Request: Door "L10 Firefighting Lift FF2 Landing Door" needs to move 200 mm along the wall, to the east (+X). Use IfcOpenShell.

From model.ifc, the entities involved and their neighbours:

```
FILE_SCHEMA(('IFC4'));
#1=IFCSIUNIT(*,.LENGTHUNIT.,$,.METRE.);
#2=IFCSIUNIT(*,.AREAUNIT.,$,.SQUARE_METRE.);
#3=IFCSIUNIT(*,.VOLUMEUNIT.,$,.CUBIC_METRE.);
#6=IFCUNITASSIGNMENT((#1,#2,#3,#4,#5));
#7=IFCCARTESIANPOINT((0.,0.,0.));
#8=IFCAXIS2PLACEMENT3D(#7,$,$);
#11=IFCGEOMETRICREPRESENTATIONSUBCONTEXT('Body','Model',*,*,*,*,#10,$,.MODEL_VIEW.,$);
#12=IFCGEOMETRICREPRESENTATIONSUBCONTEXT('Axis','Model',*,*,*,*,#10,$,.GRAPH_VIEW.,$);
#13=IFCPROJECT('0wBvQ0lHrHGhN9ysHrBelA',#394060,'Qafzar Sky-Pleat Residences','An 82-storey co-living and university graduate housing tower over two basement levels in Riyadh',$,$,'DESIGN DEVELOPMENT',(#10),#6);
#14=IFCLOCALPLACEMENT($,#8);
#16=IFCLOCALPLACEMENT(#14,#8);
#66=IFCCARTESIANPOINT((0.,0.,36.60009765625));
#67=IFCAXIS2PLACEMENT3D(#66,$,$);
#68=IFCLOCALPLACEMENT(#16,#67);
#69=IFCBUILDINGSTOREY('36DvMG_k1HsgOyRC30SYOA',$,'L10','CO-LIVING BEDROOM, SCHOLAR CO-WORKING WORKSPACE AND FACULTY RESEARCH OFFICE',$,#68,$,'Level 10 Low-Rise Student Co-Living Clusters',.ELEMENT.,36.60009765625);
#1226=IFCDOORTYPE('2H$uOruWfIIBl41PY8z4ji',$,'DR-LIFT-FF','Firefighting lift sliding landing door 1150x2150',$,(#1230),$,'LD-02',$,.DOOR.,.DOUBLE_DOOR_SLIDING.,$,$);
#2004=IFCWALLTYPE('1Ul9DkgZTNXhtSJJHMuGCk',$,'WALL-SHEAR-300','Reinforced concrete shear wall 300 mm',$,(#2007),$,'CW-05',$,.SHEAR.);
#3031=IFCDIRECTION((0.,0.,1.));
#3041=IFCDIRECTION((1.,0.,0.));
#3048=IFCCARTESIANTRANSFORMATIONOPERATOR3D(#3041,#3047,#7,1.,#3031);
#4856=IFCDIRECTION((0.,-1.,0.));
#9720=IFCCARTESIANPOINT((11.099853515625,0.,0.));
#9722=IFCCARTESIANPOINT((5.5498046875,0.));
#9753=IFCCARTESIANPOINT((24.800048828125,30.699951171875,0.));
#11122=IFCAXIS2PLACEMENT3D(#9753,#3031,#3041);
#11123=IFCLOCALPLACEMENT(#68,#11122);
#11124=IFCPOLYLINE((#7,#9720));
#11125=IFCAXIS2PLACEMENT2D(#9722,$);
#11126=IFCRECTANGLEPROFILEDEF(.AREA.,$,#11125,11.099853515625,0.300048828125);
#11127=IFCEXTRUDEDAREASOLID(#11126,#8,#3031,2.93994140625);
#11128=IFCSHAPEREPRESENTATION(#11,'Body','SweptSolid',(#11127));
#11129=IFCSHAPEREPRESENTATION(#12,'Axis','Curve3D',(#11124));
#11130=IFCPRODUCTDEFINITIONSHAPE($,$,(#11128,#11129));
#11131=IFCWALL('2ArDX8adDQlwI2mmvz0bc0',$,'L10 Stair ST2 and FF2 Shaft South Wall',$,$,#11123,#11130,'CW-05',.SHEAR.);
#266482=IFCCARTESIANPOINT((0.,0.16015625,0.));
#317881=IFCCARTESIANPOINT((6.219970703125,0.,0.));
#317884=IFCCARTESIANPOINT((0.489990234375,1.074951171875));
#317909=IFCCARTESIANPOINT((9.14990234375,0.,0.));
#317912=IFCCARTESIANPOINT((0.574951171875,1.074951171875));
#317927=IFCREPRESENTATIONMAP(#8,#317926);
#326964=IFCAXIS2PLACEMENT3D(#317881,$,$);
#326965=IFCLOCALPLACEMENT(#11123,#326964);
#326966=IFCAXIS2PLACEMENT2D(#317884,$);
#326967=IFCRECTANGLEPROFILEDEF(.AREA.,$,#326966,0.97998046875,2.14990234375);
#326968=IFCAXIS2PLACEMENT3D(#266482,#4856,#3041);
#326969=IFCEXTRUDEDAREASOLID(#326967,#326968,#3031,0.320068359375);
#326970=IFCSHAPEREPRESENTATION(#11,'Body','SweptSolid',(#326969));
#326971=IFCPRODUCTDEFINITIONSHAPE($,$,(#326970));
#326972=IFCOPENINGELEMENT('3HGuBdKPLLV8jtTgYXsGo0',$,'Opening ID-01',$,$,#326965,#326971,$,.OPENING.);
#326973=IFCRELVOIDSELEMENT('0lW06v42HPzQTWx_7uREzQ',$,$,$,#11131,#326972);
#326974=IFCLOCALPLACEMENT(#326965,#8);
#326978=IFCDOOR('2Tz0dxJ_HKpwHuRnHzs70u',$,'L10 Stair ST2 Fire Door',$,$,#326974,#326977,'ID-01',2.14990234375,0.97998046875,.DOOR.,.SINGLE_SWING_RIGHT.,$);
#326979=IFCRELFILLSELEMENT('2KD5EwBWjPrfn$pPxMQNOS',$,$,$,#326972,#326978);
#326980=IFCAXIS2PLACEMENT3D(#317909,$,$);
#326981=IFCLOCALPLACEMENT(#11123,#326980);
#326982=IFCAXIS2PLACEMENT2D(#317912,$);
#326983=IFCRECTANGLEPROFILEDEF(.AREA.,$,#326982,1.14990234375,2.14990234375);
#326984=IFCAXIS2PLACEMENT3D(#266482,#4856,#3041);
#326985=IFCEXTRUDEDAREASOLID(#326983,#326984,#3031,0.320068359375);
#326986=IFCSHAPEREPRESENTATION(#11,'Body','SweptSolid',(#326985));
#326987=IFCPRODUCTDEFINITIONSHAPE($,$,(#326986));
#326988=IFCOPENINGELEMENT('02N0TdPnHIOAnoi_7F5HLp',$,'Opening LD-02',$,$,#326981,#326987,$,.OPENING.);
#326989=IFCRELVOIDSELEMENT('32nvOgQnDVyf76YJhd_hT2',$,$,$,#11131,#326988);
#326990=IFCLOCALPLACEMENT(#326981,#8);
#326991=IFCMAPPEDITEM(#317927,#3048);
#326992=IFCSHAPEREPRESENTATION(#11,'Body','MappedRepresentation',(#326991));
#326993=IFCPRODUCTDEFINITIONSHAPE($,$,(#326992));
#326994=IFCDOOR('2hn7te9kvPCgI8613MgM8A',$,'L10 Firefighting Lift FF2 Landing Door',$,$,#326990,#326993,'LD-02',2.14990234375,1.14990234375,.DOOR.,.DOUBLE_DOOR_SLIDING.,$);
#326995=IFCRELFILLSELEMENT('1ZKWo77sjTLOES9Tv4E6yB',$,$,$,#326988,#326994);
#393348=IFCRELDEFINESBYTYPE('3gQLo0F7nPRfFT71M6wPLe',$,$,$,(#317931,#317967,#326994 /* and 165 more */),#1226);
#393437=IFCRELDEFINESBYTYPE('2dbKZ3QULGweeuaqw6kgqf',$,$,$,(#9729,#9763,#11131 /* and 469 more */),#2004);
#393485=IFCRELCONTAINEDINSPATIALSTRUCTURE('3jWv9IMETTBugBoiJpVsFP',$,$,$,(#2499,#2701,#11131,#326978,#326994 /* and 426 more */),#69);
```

```python
import ifcopenshell
import ifcopenshell.api.geometry
import ifcopenshell.util.placement
import ifcopenshell.util.unit

model = ifcopenshell.open("model.ifc")
unit_scale = ifcopenshell.util.unit.calculate_unit_scale(model)

door = model.by_guid("2hn7te9kvPCgI8613MgM8A")
opening = door.FillsVoids[0].RelatingOpeningElement
wall = opening.VoidsElements[0].RelatingBuildingElement

wall_matrix = ifcopenshell.util.placement.get_local_placement(wall.ObjectPlacement)
shift = wall_matrix[:3, 0] * 0.2 / unit_scale
before = ifcopenshell.util.placement.get_local_placement(door.ObjectPlacement)[:3, 3].copy()

# The door is placed relative to its opening, so it follows when the opening moves.
matrix = ifcopenshell.util.placement.get_local_placement(opening.ObjectPlacement)
matrix[:3, 3] += shift
ifcopenshell.api.geometry.edit_object_placement(
    model, product=opening, matrix=matrix, is_si=False, should_transform_children=True
)

after = ifcopenshell.util.placement.get_local_placement(door.ObjectPlacement)[:3, 3]
print("door moved by", (after - before).round(3) + 0.0)

model.write("model_v2.ifc")
```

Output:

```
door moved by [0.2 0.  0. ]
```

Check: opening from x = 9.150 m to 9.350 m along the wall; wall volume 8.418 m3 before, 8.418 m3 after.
